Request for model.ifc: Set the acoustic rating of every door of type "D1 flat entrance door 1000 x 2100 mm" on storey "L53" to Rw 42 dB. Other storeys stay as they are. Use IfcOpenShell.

First a look at what the model holds.

```python
import ifcopenshell
import ifcopenshell.util.element

model = ifcopenshell.open("model.ifc")
print(model.schema)
storey = next(s for s in model.by_type("IfcBuildingStorey") if s.Name == "L53")
doors = [e for e in ifcopenshell.util.element.get_decomposition(storey) if e.is_a("IfcDoor")]
seen = {}
for e in doors:
    element_type = ifcopenshell.util.element.get_type(e)
    key = (element_type.Name if element_type != e and element_type else None, ifcopenshell.util.element.get_pset(e, "Pset_DoorCommon", "AcousticRating"))
    seen[key] = seen.get(key, 0) + 1
for (name, value), count in sorted(seen.items(), key=str):
    print(count, "x", name, "|", value)
```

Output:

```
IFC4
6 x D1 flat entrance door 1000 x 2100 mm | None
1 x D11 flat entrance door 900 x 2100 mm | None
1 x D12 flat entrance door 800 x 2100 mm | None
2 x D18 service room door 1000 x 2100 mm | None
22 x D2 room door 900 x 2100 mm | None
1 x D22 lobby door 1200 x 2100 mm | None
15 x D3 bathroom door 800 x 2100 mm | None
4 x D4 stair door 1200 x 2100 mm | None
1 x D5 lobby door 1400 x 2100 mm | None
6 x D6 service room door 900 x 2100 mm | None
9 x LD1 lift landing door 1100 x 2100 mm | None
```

```python
import ifcopenshell
import ifcopenshell.api.pset
import ifcopenshell.util.element

model = ifcopenshell.open("model.ifc")

storey = next(s for s in model.by_type("IfcBuildingStorey") if s.Name == "L53")
doors = [e for e in ifcopenshell.util.element.get_decomposition(storey) if e.is_a("IfcDoor")]

count = 0
for e in doors:
    element_type = ifcopenshell.util.element.get_type(e)
    if element_type in (None, e) or element_type.Name != "D1 flat entrance door 1000 x 2100 mm":
        continue
    found = ifcopenshell.util.element.get_pset(e, "Pset_DoorCommon", should_inherit=False)
    if found:
        pset = model.by_id(found["id"])
        if len(ifcopenshell.util.element.get_elements_by_pset(pset)) > 1:
            pset = ifcopenshell.api.pset.unshare_pset(model, products=[e], pset=pset)[0]
    else:
        pset = ifcopenshell.api.pset.add_pset(model, product=e, name="Pset_DoorCommon")
    ifcopenshell.api.pset.edit_pset(model, pset=pset, properties={"AcousticRating": "Rw 42 dB"})
    count += 1

print(count, "doors updated")

model.write("model-out.ifc")
```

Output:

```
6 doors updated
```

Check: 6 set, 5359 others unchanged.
